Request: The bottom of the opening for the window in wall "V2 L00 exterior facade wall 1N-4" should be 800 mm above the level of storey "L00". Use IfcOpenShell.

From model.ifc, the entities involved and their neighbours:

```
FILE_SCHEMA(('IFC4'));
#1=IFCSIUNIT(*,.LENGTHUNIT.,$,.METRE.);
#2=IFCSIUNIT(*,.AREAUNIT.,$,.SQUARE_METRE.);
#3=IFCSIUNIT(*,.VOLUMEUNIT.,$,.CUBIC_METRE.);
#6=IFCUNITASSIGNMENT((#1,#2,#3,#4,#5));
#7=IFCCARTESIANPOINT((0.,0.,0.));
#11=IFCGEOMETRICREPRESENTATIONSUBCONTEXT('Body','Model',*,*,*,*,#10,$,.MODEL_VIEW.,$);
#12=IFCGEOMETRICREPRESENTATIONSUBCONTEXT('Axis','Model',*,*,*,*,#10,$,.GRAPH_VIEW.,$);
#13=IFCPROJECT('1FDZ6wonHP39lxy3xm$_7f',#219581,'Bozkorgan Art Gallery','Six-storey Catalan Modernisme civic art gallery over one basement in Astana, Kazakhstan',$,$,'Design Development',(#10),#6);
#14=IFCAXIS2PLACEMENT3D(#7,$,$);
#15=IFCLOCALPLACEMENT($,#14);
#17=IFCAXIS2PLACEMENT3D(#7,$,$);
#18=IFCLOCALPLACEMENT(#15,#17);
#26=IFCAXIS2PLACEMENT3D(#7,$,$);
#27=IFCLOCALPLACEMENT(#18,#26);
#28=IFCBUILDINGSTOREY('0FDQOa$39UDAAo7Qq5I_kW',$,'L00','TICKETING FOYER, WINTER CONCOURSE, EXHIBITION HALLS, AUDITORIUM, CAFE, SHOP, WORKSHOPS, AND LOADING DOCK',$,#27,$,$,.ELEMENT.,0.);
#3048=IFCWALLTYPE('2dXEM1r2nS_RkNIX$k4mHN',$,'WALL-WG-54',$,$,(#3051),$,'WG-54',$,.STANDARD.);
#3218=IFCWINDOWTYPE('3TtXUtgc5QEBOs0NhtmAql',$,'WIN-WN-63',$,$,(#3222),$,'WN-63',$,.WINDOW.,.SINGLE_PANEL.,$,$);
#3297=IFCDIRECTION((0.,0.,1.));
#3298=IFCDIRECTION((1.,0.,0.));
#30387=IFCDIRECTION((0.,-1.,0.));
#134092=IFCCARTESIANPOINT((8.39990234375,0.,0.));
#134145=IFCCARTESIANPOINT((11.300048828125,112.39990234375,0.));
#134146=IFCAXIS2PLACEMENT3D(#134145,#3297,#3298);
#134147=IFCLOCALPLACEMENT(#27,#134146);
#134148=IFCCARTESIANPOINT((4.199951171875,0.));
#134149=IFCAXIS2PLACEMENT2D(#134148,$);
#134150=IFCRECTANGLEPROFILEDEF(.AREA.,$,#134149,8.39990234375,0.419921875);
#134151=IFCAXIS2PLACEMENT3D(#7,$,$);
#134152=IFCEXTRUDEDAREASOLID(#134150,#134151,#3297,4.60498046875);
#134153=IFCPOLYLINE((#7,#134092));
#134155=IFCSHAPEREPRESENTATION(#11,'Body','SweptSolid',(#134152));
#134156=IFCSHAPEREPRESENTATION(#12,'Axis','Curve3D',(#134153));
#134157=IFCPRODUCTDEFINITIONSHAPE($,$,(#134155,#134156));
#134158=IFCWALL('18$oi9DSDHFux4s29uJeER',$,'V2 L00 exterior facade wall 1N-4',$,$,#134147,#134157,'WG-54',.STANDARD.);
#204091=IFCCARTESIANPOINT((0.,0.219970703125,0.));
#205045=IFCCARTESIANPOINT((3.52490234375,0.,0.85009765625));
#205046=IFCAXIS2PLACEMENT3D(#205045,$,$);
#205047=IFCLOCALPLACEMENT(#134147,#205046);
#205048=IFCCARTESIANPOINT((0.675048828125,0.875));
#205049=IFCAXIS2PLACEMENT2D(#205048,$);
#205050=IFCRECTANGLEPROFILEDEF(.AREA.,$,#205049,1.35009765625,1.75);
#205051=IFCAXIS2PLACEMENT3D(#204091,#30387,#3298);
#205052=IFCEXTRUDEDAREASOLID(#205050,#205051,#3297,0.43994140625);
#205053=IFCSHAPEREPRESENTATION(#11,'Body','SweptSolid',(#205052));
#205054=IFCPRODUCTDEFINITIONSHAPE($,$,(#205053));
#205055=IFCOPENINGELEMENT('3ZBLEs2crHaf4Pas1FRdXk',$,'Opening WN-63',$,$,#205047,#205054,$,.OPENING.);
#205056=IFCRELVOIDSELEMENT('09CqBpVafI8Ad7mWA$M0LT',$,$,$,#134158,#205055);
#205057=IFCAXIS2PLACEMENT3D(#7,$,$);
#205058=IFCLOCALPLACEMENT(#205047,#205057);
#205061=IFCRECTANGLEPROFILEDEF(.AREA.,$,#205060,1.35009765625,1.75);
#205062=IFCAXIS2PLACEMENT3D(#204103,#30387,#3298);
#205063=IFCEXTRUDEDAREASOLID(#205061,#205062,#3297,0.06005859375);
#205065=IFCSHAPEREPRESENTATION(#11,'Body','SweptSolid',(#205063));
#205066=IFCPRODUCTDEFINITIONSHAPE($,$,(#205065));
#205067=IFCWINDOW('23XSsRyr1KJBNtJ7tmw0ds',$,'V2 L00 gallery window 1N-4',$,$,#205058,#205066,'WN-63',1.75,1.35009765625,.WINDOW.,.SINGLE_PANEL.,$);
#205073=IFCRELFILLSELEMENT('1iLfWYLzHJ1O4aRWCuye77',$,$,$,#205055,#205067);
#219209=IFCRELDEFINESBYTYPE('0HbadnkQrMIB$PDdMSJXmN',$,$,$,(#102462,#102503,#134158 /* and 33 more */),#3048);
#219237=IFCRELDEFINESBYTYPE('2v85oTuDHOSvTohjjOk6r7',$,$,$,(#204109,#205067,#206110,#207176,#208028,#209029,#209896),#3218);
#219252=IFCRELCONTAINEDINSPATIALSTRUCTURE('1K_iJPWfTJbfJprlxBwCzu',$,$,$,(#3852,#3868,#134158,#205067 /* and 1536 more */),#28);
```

```python
import numpy as np
import ifcopenshell
import ifcopenshell.api.geometry
import ifcopenshell.geom
import ifcopenshell.util.element
import ifcopenshell.util.placement
import ifcopenshell.util.shape
import ifcopenshell.util.unit

model = ifcopenshell.open("model.ifc")
unit_scale = ifcopenshell.util.unit.calculate_unit_scale(model)

window = model.by_guid("23XSsRyr1KJBNtJ7tmw0ds")
opening = window.FillsVoids[0].RelatingOpeningElement
storey = ifcopenshell.util.element.get_container(window, ifc_class="IfcBuildingStorey")
level = ifcopenshell.util.placement.get_local_placement(storey.ObjectPlacement)[2, 3]

# The opening's origin need not be at the sill, so measure its lowest point.
shape = ifcopenshell.geom.create_shape(ifcopenshell.geom.settings(), opening)
bottom = ifcopenshell.util.shape.get_shape_bottom_elevation(shape, shape.geometry) / unit_scale
dz = level + 0.8 / unit_scale - bottom

shift = np.array([0.0, 0.0, dz])
# The window is placed relative to its opening, so it follows when the opening moves.
matrix = ifcopenshell.util.placement.get_local_placement(opening.ObjectPlacement)
matrix[:3, 3] += shift
ifcopenshell.api.geometry.edit_object_placement(
    model, product=opening, matrix=matrix, is_si=False, should_transform_children=True
)

print(f"moved by {dz * unit_scale:+.3f} m")

model.write("model_updated.ifc")
```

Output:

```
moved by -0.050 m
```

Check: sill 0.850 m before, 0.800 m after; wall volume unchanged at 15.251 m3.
